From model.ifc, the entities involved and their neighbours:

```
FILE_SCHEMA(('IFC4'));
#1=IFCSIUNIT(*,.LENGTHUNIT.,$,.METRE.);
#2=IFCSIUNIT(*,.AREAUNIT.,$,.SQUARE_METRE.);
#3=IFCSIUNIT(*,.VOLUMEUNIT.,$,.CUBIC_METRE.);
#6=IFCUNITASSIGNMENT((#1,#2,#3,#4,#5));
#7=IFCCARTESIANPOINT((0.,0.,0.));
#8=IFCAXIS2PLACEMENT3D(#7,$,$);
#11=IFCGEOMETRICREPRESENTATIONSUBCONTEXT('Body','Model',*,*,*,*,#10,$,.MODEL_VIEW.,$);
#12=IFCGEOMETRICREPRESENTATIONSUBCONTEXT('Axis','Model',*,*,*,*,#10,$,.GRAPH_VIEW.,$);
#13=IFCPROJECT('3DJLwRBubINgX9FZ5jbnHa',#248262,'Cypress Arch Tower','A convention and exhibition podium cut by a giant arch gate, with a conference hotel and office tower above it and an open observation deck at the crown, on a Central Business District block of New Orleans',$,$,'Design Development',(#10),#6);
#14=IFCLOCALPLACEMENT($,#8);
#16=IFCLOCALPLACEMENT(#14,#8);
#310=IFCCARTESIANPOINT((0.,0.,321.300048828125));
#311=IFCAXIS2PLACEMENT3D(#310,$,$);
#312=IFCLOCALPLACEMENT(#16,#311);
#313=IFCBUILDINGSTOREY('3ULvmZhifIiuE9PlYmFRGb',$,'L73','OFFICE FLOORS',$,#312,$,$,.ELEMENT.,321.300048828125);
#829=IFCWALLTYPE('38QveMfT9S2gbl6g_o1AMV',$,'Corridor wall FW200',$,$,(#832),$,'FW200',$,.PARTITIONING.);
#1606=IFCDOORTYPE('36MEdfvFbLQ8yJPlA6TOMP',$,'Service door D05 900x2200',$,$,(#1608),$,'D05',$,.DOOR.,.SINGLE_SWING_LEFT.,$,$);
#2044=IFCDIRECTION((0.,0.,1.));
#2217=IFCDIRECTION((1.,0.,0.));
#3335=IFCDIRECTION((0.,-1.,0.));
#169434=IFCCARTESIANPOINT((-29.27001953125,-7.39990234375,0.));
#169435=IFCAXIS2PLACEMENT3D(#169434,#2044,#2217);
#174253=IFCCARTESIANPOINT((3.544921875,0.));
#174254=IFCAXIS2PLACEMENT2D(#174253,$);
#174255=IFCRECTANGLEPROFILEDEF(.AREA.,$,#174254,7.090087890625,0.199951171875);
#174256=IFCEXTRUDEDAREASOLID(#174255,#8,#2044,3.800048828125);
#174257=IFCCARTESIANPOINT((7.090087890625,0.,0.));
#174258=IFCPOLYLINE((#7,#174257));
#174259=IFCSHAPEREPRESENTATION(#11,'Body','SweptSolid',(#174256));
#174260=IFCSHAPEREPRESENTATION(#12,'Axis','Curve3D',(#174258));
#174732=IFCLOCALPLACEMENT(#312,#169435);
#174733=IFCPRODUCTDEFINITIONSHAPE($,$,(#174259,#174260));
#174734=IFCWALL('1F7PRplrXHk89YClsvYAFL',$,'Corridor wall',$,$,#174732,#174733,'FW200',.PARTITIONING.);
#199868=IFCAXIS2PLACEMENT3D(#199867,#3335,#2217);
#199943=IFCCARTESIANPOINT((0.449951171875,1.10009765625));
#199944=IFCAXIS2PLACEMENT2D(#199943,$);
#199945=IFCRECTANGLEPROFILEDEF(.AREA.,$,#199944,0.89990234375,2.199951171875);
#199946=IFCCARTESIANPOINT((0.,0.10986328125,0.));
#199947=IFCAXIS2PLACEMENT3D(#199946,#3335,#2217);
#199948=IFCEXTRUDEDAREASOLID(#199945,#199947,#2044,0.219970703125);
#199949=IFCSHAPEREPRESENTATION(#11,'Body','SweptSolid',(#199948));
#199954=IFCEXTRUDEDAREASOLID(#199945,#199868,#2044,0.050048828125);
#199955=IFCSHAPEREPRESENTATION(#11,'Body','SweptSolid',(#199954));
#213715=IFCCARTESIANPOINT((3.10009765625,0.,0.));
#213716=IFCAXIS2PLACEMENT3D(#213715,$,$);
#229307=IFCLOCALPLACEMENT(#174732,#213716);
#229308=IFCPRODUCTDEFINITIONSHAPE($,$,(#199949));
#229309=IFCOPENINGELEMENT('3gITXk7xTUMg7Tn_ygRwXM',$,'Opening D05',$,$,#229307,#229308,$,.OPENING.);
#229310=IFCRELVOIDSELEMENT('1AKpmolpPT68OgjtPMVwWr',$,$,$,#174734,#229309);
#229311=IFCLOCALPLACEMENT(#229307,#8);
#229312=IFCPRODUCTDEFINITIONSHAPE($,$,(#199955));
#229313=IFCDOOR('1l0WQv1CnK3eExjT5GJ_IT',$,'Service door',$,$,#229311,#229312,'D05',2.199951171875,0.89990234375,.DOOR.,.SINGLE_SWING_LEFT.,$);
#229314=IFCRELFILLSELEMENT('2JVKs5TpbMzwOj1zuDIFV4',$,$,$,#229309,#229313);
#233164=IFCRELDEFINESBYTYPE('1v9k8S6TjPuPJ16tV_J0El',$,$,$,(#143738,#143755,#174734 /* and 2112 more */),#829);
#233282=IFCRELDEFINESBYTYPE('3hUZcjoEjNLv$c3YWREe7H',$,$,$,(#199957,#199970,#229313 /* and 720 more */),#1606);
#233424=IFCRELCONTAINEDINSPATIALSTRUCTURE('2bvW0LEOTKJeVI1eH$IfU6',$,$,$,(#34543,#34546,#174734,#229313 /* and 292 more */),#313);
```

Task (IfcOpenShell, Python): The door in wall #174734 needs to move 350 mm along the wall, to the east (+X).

```python
import ifcopenshell
import ifcopenshell.api.geometry
import ifcopenshell.util.placement

model = ifcopenshell.open("model.ifc")

door = model.by_id(229313)
opening = door.FillsVoids[0].RelatingOpeningElement
wall = opening.VoidsElements[0].RelatingBuildingElement

wall_matrix = ifcopenshell.util.placement.get_local_placement(wall.ObjectPlacement)
shift = wall_matrix[:3, 0] * 0.35
before = ifcopenshell.util.placement.get_local_placement(door.ObjectPlacement)[:3, 3].copy()

# The door is placed relative to its opening, so it follows when the opening moves.
matrix = ifcopenshell.util.placement.get_local_placement(opening.ObjectPlacement)
matrix[:3, 3] += shift
ifcopenshell.api.geometry.edit_object_placement(
    model, product=opening, matrix=matrix, is_si=False, should_transform_children=True
)

after = ifcopenshell.util.placement.get_local_placement(door.ObjectPlacement)[:3, 3]
print("door moved by", (after - before).round(3) + 0.0)

model.write("model_edited.ifc")
```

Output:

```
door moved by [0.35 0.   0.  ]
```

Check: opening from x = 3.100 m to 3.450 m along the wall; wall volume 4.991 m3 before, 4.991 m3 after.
